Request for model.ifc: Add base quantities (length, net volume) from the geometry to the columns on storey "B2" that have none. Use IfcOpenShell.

First a look at what the model holds.

```python
import ifcopenshell
import ifcopenshell.util.element
import ifcopenshell.util.unit

model = ifcopenshell.open("model.ifc")
print(model.schema)
for unit_type in ("LENGTHUNIT", "AREAUNIT", "VOLUMEUNIT"):
    print(unit_type, ifcopenshell.util.unit.calculate_unit_scale(model, unit_type))
storey = next(s for s in model.by_type("IfcBuildingStorey") if s.Name == "B2")
columns = [e for e in ifcopenshell.util.element.get_decomposition(storey) if e.is_a("IfcColumn")]
for e in sorted(columns, key=lambda e: e.id()):
    print(e.id(), e.is_a(), e.Name, list(ifcopenshell.util.element.get_psets(e, qtos_only=True)), sep=" | ")
```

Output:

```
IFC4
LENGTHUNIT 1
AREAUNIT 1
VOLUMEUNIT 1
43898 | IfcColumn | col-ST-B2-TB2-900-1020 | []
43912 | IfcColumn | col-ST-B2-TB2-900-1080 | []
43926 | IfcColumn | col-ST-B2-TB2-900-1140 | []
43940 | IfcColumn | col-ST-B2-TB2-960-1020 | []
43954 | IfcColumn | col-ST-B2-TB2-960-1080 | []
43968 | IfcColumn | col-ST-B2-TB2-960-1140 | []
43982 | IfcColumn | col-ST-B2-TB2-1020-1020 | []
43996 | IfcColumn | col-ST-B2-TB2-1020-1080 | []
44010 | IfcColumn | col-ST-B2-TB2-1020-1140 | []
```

```python
import ifcopenshell
import ifcopenshell.api.pset
import ifcopenshell.geom
import ifcopenshell.util.element
import ifcopenshell.util.shape
import ifcopenshell.util.unit

model = ifcopenshell.open("model.ifc")
unit_scale = ifcopenshell.util.unit.calculate_unit_scale(model)
volume_scale = ifcopenshell.util.unit.calculate_unit_scale(model, "VOLUMEUNIT")
settings = ifcopenshell.geom.settings()

storey = next(s for s in model.by_type("IfcBuildingStorey") if s.Name == "B2")
columns = [e for e in ifcopenshell.util.element.get_decomposition(storey) if e.is_a("IfcColumn")]

for e in sorted(columns, key=lambda e: e.id()):
    if ifcopenshell.util.element.get_psets(e, qtos_only=True, should_inherit=False):
        continue
    # Geometry comes back in metres, in the element's own axes.
    shape = ifcopenshell.geom.create_shape(settings, e)
    values = {
        "Length": ifcopenshell.util.shape.get_z(shape.geometry) / unit_scale,
        "NetVolume": ifcopenshell.util.shape.get_volume(shape.geometry) / volume_scale,
    }
    qto = ifcopenshell.api.pset.add_qto(model, product=e, name="Qto_ColumnBaseQuantities")
    ifcopenshell.api.pset.edit_qto(model, qto=qto, properties=values)
    print(e.id(), {k: round(v, 3) for k, v in values.items()})

model.write("model-out.ifc")
```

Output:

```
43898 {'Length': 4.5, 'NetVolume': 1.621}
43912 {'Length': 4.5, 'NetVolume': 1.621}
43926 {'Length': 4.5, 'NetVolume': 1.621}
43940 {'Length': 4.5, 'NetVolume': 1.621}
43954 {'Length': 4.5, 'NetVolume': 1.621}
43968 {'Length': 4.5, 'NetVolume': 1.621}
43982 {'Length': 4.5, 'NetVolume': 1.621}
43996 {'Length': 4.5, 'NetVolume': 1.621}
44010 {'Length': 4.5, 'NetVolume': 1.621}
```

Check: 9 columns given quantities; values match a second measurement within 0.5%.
